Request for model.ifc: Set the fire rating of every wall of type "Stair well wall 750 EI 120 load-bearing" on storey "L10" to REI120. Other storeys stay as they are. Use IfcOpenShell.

First a look at what the model holds.

```python
import ifcopenshell
import ifcopenshell.util.element

model = ifcopenshell.open("model.ifc")
print(model.schema)
storey = next(s for s in model.by_type("IfcBuildingStorey") if s.Name == "L10")
walls = [e for e in ifcopenshell.util.element.get_decomposition(storey) if e.is_a("IfcWall")]
seen = {}
for e in walls:
    element_type = ifcopenshell.util.element.get_type(e)
    key = (element_type.Name if element_type != e and element_type else None, ifcopenshell.util.element.get_pset(e, "Pset_WallCommon", "FireRating"))
    seen[key] = seen.get(key, 0) + 1
for (name, value), count in sorted(seen.items(), key=str):
    print(count, "x", name, "|", value)
```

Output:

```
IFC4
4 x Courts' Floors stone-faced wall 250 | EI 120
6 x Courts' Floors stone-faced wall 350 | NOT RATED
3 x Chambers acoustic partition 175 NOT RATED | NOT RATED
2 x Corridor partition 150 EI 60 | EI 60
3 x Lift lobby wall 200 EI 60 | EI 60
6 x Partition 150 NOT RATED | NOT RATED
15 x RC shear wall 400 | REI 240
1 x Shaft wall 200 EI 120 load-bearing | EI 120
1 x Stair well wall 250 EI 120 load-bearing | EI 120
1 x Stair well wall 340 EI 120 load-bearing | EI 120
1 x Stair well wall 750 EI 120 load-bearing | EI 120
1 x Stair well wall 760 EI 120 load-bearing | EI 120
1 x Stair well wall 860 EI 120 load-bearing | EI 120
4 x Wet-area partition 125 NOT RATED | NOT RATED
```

```python
import ifcopenshell
import ifcopenshell.api.pset
import ifcopenshell.util.element

model = ifcopenshell.open("model.ifc")

storey = next(s for s in model.by_type("IfcBuildingStorey") if s.Name == "L10")
walls = [e for e in ifcopenshell.util.element.get_decomposition(storey) if e.is_a("IfcWall")]

count = 0
for e in walls:
    element_type = ifcopenshell.util.element.get_type(e)
    if element_type in (None, e) or element_type.Name != "Stair well wall 750 EI 120 load-bearing":
        continue
    # add_pset returns the element's existing set when there is one.
    pset = ifcopenshell.api.pset.add_pset(model, product=e, name="Pset_WallCommon")
    ifcopenshell.api.pset.edit_pset(model, pset=pset, properties={"FireRating": "REI120"})
    count += 1

print(count, "walls updated")

model.write("model_updated.ifc")
```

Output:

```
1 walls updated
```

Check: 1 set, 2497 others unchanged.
